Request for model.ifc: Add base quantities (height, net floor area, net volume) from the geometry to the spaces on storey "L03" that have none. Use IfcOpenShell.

First a look at what the model holds.

```python
import ifcopenshell
import ifcopenshell.util.element
import ifcopenshell.util.unit

model = ifcopenshell.open("model.ifc")
print(model.schema)
for unit_type in ("LENGTHUNIT", "AREAUNIT", "VOLUMEUNIT"):
    print(unit_type, ifcopenshell.util.unit.calculate_unit_scale(model, unit_type))
storey = next(s for s in model.by_type("IfcBuildingStorey") if s.Name == "L03")
spaces = [e for e in ifcopenshell.util.element.get_decomposition(storey) if e.is_a("IfcSpace")]
for e in sorted(spaces, key=lambda e: e.id()):
    print(e.id(), e.is_a(), e.Name, list(ifcopenshell.util.element.get_psets(e, qtos_only=True)), sep=" | ")
```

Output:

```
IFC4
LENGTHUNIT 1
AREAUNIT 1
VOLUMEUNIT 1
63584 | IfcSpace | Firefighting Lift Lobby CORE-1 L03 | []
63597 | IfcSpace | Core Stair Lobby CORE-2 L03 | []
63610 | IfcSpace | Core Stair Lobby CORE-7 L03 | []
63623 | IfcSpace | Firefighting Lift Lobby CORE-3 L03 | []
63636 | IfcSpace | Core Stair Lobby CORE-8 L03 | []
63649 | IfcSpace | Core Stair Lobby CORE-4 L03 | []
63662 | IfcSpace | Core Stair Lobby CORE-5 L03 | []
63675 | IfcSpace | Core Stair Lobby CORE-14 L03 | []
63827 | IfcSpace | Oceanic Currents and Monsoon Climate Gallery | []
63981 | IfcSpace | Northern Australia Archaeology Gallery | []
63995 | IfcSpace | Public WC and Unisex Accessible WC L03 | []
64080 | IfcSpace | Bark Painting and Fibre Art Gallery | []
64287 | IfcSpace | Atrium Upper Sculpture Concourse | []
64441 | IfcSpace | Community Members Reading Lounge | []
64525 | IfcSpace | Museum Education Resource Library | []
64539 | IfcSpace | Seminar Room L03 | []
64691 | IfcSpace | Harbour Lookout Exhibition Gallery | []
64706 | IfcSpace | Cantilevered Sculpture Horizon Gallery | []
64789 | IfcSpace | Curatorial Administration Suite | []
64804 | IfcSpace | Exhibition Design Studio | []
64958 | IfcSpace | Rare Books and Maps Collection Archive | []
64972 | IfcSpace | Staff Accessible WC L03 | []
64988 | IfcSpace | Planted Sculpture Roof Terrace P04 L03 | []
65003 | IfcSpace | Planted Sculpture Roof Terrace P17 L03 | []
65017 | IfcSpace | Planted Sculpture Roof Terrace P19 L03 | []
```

```python
import ifcopenshell
import ifcopenshell.api.pset
import ifcopenshell.geom
import ifcopenshell.util.element
import ifcopenshell.util.shape
import ifcopenshell.util.unit

model = ifcopenshell.open("model.ifc")
unit_scale = ifcopenshell.util.unit.calculate_unit_scale(model)
area_scale = ifcopenshell.util.unit.calculate_unit_scale(model, "AREAUNIT")
volume_scale = ifcopenshell.util.unit.calculate_unit_scale(model, "VOLUMEUNIT")
settings = ifcopenshell.geom.settings()

storey = next(s for s in model.by_type("IfcBuildingStorey") if s.Name == "L03")
spaces = [e for e in ifcopenshell.util.element.get_decomposition(storey) if e.is_a("IfcSpace")]

for e in sorted(spaces, key=lambda e: e.id()):
    if ifcopenshell.util.element.get_psets(e, qtos_only=True, should_inherit=False):
        continue
    # Geometry comes back in metres, in the element's own axes.
    shape = ifcopenshell.geom.create_shape(settings, e)
    values = {
        "Height": ifcopenshell.util.shape.get_z(shape.geometry) / unit_scale,
        "NetFloorArea": ifcopenshell.util.shape.get_footprint_area(shape.geometry) / area_scale,
        "NetVolume": ifcopenshell.util.shape.get_volume(shape.geometry) / volume_scale,
    }
    qto = ifcopenshell.api.pset.add_qto(model, product=e, name="Qto_SpaceBaseQuantities")
    ifcopenshell.api.pset.edit_qto(model, qto=qto, properties=values)
    print(e.id(), {k: round(v, 3) for k, v in values.items()})

model.write("model_updated.ifc")
```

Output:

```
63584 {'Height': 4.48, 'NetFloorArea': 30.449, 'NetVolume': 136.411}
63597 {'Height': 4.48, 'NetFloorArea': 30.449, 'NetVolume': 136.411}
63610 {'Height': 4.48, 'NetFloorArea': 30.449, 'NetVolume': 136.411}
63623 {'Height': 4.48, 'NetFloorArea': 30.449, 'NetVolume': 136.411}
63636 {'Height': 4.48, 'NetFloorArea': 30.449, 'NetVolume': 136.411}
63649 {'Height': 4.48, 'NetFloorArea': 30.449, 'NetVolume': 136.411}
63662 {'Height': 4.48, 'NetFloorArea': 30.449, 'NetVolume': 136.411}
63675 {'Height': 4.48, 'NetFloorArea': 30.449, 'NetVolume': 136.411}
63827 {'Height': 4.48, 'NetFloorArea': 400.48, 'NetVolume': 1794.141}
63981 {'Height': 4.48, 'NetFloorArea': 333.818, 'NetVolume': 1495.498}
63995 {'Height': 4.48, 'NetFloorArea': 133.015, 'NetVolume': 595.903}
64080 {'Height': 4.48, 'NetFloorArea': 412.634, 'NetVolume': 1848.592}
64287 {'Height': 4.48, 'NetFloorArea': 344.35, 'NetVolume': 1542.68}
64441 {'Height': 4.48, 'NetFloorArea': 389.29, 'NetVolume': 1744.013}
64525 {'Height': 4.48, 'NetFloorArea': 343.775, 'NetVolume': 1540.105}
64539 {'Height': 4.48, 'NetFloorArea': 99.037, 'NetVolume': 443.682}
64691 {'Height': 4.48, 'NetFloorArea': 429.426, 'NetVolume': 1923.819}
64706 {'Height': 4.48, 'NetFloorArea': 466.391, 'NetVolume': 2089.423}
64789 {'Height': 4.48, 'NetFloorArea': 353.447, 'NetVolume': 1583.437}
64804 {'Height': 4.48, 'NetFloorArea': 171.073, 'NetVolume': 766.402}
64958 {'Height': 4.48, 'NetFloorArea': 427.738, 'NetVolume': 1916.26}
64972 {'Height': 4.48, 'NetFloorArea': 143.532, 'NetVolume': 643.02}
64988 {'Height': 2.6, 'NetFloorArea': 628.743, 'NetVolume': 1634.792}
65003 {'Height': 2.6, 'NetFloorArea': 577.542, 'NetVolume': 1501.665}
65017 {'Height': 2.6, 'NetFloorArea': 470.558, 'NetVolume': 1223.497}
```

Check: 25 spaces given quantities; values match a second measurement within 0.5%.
